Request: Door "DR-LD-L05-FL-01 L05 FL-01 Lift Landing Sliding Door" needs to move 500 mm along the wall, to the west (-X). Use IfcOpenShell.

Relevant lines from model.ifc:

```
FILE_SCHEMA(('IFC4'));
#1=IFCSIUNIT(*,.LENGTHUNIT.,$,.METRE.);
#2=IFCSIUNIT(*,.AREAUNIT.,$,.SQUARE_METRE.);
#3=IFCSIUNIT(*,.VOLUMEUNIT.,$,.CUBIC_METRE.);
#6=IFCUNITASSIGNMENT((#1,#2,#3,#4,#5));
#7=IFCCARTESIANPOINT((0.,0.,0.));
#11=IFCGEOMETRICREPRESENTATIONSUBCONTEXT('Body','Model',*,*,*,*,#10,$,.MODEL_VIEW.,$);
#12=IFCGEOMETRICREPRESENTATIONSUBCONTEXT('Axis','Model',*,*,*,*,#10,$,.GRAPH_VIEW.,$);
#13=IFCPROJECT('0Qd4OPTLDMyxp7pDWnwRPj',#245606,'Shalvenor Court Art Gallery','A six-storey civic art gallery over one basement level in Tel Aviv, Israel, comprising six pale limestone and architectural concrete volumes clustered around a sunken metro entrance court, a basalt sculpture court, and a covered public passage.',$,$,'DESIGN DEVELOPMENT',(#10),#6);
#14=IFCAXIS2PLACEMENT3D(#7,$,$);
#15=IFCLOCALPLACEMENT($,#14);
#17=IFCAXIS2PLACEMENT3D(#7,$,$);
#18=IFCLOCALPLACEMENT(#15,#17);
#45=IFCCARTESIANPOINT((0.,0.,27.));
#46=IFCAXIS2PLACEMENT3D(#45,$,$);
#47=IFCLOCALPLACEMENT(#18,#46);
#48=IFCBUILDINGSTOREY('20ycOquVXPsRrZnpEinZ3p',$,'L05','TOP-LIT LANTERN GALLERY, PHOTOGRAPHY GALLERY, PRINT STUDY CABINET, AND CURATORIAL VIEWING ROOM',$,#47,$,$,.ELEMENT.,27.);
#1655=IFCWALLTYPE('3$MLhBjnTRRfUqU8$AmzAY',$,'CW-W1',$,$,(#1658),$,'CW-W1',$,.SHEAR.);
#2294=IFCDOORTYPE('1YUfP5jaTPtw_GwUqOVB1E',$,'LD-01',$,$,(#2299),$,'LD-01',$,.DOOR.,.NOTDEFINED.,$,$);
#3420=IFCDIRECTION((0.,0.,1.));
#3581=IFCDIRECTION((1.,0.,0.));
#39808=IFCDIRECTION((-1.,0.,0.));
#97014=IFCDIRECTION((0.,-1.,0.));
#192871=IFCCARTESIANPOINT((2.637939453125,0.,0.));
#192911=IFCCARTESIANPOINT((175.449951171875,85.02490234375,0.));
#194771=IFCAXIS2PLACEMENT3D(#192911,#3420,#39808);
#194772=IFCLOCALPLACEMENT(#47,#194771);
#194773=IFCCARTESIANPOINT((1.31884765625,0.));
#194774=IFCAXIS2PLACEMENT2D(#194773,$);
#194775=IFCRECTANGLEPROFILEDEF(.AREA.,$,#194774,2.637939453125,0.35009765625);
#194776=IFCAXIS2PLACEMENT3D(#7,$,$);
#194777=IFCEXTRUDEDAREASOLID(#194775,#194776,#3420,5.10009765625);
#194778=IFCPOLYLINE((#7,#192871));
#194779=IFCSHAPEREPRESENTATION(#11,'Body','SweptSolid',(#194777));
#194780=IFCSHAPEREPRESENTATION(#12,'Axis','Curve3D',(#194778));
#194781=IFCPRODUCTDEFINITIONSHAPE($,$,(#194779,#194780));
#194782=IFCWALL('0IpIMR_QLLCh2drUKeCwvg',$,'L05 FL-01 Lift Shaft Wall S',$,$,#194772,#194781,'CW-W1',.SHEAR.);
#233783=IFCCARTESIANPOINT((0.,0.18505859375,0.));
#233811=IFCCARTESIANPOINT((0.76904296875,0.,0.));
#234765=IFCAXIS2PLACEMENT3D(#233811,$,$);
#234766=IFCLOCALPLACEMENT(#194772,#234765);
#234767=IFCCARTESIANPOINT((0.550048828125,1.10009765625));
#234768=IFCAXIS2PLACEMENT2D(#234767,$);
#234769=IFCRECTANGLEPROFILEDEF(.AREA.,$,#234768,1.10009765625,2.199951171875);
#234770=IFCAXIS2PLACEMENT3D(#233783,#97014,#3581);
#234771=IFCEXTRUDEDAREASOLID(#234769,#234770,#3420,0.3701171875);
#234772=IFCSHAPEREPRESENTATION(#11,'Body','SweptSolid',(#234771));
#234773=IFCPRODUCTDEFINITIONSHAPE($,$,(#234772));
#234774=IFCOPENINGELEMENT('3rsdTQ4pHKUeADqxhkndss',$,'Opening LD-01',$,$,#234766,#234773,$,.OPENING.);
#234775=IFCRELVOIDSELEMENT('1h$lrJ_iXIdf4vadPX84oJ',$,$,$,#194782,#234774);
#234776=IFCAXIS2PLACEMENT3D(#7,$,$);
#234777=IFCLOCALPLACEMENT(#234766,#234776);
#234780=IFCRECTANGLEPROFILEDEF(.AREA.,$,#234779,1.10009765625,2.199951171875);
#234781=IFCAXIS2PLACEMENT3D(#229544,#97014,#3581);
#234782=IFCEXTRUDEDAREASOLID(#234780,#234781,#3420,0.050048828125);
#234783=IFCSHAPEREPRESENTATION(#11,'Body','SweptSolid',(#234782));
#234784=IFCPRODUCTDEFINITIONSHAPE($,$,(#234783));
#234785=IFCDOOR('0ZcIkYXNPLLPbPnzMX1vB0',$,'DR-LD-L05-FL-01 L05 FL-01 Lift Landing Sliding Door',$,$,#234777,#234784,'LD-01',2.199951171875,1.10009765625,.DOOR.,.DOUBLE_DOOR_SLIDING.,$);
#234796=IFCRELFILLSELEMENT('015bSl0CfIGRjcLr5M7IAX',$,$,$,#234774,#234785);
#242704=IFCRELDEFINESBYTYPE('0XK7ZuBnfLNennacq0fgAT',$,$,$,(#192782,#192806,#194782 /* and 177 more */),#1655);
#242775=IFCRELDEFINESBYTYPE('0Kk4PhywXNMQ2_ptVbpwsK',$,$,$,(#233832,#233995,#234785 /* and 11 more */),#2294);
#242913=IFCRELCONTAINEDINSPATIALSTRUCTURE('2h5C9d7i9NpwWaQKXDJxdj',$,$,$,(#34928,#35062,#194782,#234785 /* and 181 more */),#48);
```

```python
import ifcopenshell
import ifcopenshell.api.geometry
import ifcopenshell.util.placement
import ifcopenshell.util.unit

model = ifcopenshell.open("model.ifc")
unit_scale = ifcopenshell.util.unit.calculate_unit_scale(model)

door = model.by_id(234785)
opening = door.FillsVoids[0].RelatingOpeningElement
wall = opening.VoidsElements[0].RelatingBuildingElement

wall_matrix = ifcopenshell.util.placement.get_local_placement(wall.ObjectPlacement)
shift = wall_matrix[:3, 0] * 0.5 / unit_scale
before = ifcopenshell.util.placement.get_local_placement(door.ObjectPlacement)[:3, 3].copy()

# The door is placed relative to its opening, so it follows when the opening moves.
matrix = ifcopenshell.util.placement.get_local_placement(opening.ObjectPlacement)
matrix[:3, 3] += shift
ifcopenshell.api.geometry.edit_object_placement(
    model, product=opening, matrix=matrix, is_si=False, should_transform_children=True
)

after = ifcopenshell.util.placement.get_local_placement(door.ObjectPlacement)[:3, 3]
print("door moved by", (after - before).round(3) + 0.0)

model.write("model_rev.ifc")
```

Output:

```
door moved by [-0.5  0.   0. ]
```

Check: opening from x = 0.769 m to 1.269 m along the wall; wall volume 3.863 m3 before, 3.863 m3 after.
